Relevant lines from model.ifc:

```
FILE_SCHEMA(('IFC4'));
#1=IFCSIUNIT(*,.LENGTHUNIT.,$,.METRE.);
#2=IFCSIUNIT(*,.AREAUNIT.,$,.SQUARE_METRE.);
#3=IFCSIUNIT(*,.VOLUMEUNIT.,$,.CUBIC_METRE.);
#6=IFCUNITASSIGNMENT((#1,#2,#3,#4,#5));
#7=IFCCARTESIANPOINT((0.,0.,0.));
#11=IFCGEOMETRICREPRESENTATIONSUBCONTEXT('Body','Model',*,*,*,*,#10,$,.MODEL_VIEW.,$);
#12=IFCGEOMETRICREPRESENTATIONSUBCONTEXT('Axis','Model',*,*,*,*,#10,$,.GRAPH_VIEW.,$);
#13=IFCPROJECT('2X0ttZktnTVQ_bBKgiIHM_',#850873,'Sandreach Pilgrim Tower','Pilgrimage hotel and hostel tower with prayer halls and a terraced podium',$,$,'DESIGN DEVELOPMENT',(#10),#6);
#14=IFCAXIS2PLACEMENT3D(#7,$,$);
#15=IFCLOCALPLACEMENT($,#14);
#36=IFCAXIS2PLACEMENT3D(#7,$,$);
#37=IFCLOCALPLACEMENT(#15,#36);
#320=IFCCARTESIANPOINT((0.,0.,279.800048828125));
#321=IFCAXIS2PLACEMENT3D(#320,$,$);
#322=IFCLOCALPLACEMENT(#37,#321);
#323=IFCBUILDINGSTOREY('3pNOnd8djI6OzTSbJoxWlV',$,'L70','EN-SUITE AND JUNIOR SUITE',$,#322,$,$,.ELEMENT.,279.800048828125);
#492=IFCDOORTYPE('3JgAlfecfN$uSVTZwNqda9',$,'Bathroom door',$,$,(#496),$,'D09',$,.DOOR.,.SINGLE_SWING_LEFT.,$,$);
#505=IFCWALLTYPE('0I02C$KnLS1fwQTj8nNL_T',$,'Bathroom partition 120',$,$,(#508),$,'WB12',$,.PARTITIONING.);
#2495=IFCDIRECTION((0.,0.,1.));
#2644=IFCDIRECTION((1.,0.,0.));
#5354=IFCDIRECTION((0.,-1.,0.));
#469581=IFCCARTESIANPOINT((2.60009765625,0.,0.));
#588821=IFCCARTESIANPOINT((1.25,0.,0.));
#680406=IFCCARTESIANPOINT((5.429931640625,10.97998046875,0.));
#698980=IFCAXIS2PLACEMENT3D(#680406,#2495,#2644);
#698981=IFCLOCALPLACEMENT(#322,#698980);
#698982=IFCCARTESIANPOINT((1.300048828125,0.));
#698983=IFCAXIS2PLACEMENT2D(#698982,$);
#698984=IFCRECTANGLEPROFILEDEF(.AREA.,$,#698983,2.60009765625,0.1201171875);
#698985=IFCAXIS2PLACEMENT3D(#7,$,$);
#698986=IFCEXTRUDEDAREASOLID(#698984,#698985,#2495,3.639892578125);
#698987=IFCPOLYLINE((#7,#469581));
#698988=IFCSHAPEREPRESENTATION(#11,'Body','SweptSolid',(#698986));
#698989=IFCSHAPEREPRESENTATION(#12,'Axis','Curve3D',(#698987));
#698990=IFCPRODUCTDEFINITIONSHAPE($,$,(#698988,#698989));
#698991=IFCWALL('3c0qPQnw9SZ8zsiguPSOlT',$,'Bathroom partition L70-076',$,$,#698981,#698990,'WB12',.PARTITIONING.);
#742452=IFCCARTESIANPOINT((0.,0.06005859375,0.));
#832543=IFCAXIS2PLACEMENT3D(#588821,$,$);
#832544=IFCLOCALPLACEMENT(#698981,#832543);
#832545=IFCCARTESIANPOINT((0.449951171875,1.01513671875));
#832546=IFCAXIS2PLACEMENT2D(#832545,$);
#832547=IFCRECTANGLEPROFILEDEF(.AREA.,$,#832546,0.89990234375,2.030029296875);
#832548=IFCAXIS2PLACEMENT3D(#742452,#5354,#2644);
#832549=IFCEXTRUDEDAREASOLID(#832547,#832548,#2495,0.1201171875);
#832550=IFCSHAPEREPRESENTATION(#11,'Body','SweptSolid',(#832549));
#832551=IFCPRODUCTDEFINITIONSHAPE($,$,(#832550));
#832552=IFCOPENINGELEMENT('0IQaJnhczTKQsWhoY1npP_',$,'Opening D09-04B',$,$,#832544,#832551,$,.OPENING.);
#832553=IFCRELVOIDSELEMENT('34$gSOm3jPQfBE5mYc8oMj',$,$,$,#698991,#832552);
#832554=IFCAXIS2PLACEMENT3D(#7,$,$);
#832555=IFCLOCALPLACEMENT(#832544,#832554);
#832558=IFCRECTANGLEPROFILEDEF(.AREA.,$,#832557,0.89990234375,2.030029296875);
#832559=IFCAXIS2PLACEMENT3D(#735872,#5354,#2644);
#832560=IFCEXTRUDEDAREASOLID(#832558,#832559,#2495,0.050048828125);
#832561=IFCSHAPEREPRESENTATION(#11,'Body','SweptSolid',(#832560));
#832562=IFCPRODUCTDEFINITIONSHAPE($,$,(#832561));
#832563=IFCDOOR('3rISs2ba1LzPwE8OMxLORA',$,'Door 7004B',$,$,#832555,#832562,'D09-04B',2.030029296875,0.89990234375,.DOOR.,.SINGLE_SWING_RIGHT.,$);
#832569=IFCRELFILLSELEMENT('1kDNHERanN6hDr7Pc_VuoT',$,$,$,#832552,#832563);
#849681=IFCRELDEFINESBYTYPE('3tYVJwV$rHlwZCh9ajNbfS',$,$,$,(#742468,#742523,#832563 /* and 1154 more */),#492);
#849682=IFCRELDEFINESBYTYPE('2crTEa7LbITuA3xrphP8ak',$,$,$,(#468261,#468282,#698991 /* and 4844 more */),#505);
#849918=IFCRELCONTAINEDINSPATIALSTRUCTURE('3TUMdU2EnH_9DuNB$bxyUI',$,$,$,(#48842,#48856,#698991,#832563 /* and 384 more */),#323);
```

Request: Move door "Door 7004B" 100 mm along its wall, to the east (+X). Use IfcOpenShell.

```python
import ifcopenshell
import ifcopenshell.api.geometry
import ifcopenshell.util.placement
import ifcopenshell.util.unit

model = ifcopenshell.open("model.ifc")
unit_scale = ifcopenshell.util.unit.calculate_unit_scale(model)

door = model.by_guid("3rISs2ba1LzPwE8OMxLORA")
opening = door.FillsVoids[0].RelatingOpeningElement
wall = opening.VoidsElements[0].RelatingBuildingElement

wall_matrix = ifcopenshell.util.placement.get_local_placement(wall.ObjectPlacement)
shift = wall_matrix[:3, 0] * 0.1 / unit_scale
before = ifcopenshell.util.placement.get_local_placement(door.ObjectPlacement)[:3, 3].copy()

# The door is placed relative to its opening, so it follows when the opening moves.
matrix = ifcopenshell.util.placement.get_local_placement(opening.ObjectPlacement)
matrix[:3, 3] += shift
ifcopenshell.api.geometry.edit_object_placement(
    model, product=opening, matrix=matrix, is_si=False, should_transform_children=True
)

after = ifcopenshell.util.placement.get_local_placement(door.ObjectPlacement)[:3, 3]
print("door moved by", (after - before).round(3) + 0.0)

model.write("model-out.ifc")
```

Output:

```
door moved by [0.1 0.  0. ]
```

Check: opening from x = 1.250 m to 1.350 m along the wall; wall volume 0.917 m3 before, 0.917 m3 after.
